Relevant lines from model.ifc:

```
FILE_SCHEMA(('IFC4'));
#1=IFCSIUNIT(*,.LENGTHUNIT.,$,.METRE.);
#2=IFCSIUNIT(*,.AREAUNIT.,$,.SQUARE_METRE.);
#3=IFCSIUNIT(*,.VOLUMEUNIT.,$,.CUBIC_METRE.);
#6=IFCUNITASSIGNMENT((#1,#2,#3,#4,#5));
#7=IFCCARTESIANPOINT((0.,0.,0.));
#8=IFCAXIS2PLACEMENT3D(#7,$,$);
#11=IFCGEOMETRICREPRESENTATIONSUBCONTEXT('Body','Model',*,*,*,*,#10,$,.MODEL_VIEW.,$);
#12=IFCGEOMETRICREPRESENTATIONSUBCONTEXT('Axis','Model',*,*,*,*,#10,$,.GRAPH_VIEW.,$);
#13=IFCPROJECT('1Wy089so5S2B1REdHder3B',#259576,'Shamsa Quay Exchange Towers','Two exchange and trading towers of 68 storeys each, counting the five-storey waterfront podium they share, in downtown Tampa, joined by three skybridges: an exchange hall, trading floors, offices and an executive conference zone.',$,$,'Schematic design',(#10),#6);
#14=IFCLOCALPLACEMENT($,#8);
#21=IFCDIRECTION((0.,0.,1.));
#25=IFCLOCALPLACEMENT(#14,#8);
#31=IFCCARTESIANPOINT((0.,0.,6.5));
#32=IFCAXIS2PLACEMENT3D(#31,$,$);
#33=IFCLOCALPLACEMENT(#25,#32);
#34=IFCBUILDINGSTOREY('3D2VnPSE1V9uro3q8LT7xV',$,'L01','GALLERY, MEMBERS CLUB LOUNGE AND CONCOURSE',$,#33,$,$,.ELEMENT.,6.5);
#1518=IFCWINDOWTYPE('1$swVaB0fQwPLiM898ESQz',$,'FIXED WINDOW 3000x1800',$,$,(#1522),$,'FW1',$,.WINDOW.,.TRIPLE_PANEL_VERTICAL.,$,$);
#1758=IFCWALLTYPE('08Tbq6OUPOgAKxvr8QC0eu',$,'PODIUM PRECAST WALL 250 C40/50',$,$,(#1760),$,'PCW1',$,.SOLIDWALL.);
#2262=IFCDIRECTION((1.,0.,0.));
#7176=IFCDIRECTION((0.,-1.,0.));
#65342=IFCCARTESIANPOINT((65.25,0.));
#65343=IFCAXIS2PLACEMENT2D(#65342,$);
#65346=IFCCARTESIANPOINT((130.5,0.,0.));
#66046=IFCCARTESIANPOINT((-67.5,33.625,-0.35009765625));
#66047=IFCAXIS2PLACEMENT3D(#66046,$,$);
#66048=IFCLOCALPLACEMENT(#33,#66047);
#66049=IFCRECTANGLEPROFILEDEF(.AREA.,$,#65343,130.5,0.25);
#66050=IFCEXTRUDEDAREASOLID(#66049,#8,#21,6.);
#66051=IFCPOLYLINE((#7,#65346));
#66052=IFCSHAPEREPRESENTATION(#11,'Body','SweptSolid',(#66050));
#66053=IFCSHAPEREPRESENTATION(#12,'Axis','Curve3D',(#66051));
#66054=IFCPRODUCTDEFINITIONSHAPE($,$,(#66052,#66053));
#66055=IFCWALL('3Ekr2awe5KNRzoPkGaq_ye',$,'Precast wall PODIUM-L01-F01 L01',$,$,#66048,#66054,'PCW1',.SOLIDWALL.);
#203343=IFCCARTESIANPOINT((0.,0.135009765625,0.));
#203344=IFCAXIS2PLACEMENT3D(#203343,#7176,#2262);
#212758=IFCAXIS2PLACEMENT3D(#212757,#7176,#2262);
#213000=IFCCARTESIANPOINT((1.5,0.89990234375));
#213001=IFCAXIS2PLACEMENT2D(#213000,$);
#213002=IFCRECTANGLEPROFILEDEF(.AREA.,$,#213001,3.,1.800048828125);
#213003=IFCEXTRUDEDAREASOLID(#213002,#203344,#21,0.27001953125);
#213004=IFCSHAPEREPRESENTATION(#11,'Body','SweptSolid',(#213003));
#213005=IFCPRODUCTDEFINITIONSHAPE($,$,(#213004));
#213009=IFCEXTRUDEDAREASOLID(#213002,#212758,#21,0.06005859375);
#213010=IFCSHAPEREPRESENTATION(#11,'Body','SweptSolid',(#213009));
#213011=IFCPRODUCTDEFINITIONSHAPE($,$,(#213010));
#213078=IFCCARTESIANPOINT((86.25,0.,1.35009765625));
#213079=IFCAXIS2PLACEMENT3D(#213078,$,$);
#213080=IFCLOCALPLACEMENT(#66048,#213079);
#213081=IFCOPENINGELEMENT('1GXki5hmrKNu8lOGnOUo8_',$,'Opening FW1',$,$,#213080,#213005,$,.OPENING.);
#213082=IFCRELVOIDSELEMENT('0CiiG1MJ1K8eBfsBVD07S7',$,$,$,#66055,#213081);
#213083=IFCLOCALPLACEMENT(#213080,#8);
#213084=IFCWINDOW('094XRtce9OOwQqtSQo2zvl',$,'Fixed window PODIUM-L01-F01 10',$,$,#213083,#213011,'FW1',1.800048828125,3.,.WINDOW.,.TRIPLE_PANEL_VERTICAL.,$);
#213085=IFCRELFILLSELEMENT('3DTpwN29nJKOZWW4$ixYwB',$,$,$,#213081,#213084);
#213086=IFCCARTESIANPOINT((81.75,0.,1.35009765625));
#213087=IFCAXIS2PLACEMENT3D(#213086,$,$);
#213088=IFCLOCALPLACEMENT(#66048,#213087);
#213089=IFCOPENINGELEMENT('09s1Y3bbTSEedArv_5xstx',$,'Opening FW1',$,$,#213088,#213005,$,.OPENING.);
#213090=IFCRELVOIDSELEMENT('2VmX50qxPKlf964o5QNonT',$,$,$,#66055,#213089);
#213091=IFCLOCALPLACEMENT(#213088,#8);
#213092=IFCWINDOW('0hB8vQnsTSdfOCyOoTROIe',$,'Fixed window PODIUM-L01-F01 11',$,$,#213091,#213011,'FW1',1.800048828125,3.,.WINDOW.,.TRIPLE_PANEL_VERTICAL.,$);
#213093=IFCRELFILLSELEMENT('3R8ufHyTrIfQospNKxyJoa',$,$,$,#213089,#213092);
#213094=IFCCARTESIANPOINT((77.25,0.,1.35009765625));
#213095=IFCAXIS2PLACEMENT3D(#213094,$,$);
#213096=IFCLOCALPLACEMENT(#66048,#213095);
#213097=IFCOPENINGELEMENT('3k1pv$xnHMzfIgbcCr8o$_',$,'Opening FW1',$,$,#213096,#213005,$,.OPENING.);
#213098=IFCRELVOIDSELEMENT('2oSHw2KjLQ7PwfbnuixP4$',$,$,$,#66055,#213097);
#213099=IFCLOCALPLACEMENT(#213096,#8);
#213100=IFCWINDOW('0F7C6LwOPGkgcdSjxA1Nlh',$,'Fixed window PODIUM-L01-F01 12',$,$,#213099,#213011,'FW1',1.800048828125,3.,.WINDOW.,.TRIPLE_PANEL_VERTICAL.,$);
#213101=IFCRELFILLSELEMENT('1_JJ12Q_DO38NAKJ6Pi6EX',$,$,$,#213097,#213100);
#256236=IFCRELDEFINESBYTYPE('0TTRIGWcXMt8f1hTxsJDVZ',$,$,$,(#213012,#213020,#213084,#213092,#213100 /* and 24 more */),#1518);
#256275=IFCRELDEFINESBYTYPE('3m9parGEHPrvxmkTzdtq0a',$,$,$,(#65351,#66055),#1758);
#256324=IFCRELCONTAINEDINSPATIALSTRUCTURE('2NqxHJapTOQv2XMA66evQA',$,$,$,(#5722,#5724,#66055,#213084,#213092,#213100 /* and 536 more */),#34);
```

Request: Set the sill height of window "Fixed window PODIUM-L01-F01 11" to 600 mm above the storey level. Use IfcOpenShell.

```python
import numpy as np
import ifcopenshell
import ifcopenshell.api.geometry
import ifcopenshell.geom
import ifcopenshell.util.element
import ifcopenshell.util.placement
import ifcopenshell.util.shape
import ifcopenshell.util.unit

model = ifcopenshell.open("model.ifc")
unit_scale = ifcopenshell.util.unit.calculate_unit_scale(model)

window = model.by_guid("0hB8vQnsTSdfOCyOoTROIe")
opening = window.FillsVoids[0].RelatingOpeningElement
storey = ifcopenshell.util.element.get_container(window, ifc_class="IfcBuildingStorey")
level = ifcopenshell.util.placement.get_local_placement(storey.ObjectPlacement)[2, 3]

# The opening's origin need not be at the sill, so measure its lowest point.
shape = ifcopenshell.geom.create_shape(ifcopenshell.geom.settings(), opening)
bottom = ifcopenshell.util.shape.get_shape_bottom_elevation(shape, shape.geometry) / unit_scale
dz = level + 0.6 / unit_scale - bottom

shift = np.array([0.0, 0.0, dz])
# The window is placed relative to its opening, so it follows when the opening moves.
matrix = ifcopenshell.util.placement.get_local_placement(opening.ObjectPlacement)
matrix[:3, 3] += shift
ifcopenshell.api.geometry.edit_object_placement(
    model, product=opening, matrix=matrix, is_si=False, should_transform_children=True
)

print(f"moved by {dz * unit_scale:+.3f} m")

model.write("model_updated.ifc")
```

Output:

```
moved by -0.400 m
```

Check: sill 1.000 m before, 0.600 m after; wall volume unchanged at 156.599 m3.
